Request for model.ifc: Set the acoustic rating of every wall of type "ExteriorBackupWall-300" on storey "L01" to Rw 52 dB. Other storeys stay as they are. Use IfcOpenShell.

First a look at what the model holds.

```python
import ifcopenshell
import ifcopenshell.util.element

model = ifcopenshell.open("model.ifc")
print(model.schema)
storey = next(s for s in model.by_type("IfcBuildingStorey") if s.Name == "L01")
walls = [e for e in ifcopenshell.util.element.get_decomposition(storey) if e.is_a("IfcWall")]
seen = {}
for e in walls:
    element_type = ifcopenshell.util.element.get_type(e)
    key = (element_type.Name if element_type != e and element_type else None, ifcopenshell.util.element.get_pset(e, "Pset_WallCommon", "AcousticRating"))
    seen[key] = seen.get(key, 0) + 1
for (name, value), count in sorted(seen.items(), key=str):
    print(count, "x", name, "|", value)
```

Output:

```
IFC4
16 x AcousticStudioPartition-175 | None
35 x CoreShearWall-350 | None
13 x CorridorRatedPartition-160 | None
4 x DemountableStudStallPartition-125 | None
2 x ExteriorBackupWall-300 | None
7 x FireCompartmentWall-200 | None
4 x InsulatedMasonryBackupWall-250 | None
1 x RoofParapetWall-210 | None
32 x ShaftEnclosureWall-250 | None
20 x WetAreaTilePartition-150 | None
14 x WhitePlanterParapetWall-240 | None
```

```python
import ifcopenshell
import ifcopenshell.api.pset
import ifcopenshell.util.element

model = ifcopenshell.open("model.ifc")

storey = next(s for s in model.by_type("IfcBuildingStorey") if s.Name == "L01")
walls = [e for e in ifcopenshell.util.element.get_decomposition(storey) if e.is_a("IfcWall")]

count = 0
for e in walls:
    element_type = ifcopenshell.util.element.get_type(e)
    if element_type in (None, e) or element_type.Name != "ExteriorBackupWall-300":
        continue
    # add_pset returns the element's existing set when there is one.
    pset = ifcopenshell.api.pset.add_pset(model, product=e, name="Pset_WallCommon")
    ifcopenshell.api.pset.edit_pset(model, pset=pset, properties={"AcousticRating": "Rw 52 dB"})
    count += 1

print(count, "walls updated")

model.write("model_v2.ifc")
```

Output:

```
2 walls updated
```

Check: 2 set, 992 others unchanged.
